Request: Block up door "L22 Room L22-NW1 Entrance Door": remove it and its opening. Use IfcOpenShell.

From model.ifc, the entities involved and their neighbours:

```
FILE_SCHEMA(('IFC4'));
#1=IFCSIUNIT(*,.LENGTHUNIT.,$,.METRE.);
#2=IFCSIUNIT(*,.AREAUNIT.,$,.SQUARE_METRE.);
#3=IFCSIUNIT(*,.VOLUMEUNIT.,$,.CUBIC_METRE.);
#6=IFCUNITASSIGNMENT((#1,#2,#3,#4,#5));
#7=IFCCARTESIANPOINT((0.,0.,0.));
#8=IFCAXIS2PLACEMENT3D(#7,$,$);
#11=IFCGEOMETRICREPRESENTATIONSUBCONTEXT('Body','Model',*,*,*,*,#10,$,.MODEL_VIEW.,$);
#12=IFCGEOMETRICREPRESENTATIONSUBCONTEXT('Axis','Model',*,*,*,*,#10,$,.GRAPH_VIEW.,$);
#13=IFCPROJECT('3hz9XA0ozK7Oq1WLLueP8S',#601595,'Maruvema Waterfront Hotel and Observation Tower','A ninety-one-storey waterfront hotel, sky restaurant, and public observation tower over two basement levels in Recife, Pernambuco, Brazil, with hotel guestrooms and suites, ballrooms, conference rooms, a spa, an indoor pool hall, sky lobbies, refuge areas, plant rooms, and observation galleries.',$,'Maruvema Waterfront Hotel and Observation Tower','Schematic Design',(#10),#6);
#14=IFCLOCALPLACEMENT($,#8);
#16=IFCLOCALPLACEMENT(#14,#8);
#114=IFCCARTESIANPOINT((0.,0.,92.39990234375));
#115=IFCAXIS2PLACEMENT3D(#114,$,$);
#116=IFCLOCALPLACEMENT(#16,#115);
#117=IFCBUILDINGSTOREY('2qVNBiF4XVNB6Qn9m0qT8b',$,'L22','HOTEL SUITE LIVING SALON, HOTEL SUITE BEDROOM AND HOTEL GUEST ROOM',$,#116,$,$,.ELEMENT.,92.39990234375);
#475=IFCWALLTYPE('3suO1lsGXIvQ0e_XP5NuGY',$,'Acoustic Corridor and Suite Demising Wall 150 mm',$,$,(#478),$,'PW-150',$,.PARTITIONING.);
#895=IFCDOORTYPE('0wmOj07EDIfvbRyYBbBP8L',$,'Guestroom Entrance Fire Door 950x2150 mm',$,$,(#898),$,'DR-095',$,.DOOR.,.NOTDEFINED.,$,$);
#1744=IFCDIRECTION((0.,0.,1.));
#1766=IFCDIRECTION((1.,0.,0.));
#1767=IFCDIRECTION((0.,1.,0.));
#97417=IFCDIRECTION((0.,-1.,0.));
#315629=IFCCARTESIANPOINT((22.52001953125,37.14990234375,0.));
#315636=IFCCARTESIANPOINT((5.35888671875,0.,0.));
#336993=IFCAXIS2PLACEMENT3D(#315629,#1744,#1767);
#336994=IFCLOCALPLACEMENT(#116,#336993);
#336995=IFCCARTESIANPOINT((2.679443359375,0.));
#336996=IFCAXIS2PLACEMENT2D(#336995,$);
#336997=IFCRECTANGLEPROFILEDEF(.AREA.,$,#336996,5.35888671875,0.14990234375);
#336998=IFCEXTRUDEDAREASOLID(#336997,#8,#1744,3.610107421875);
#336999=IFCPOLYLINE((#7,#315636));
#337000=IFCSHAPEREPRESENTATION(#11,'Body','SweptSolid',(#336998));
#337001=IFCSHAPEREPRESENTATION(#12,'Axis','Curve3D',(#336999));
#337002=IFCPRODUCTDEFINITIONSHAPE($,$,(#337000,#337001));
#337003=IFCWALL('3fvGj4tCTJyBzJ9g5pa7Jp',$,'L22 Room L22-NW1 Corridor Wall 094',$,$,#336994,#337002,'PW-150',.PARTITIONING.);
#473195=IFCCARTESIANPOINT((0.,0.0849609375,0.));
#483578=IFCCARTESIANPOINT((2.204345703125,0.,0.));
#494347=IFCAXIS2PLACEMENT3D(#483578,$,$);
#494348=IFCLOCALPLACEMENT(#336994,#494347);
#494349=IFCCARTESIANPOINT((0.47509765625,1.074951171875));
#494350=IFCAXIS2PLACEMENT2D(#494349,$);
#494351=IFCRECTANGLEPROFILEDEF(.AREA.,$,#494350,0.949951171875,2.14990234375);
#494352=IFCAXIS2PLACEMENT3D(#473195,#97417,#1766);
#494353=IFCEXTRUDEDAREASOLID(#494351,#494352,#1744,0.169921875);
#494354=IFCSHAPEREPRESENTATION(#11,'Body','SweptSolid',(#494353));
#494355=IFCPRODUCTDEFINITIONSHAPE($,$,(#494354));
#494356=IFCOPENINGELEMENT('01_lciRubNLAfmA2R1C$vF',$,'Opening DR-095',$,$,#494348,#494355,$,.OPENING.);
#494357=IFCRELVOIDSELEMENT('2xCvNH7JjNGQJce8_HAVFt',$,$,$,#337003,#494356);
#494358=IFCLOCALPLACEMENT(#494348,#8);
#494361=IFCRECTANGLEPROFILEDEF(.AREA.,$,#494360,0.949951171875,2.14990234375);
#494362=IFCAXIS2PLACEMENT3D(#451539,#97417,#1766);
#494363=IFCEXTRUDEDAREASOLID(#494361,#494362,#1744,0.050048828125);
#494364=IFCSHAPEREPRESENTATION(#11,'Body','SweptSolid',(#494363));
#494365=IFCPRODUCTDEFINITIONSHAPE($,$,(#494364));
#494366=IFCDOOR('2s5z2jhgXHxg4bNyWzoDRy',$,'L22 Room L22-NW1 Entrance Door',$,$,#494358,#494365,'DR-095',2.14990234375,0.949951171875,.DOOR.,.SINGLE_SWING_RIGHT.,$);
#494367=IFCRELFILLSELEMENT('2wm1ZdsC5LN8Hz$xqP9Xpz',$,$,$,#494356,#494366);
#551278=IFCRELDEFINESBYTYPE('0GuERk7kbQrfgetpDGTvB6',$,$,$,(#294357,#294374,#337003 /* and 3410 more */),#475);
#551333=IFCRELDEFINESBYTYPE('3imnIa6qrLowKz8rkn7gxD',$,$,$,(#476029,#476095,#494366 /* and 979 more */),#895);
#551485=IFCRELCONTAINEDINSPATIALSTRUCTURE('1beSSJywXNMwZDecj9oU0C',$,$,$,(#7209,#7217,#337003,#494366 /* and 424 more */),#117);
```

```python
import ifcopenshell
import ifcopenshell.api.feature
import ifcopenshell.api.root
import ifcopenshell.geom
import ifcopenshell.util.shape

model = ifcopenshell.open("model.ifc")
settings = ifcopenshell.geom.settings()


def volume(element):
    """Net volume in cubic metres, openings subtracted."""
    shape = ifcopenshell.geom.create_shape(settings, element)
    return ifcopenshell.util.shape.get_volume(shape.geometry)


door = model.by_guid("2s5z2jhgXHxg4bNyWzoDRy")
opening = door.FillsVoids[0].RelatingOpeningElement
wall = opening.VoidsElements[0].RelatingBuildingElement
before = volume(wall)

ifcopenshell.api.root.remove_product(model, product=door)
ifcopenshell.api.feature.remove_feature(model, feature=opening)

after = volume(wall)

print(f"wall volume {before:.3f} -> {after:.3f} m3")

model.write("model_rev.ifc")
```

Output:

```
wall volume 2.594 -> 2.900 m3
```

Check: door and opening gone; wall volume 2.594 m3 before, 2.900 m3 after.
